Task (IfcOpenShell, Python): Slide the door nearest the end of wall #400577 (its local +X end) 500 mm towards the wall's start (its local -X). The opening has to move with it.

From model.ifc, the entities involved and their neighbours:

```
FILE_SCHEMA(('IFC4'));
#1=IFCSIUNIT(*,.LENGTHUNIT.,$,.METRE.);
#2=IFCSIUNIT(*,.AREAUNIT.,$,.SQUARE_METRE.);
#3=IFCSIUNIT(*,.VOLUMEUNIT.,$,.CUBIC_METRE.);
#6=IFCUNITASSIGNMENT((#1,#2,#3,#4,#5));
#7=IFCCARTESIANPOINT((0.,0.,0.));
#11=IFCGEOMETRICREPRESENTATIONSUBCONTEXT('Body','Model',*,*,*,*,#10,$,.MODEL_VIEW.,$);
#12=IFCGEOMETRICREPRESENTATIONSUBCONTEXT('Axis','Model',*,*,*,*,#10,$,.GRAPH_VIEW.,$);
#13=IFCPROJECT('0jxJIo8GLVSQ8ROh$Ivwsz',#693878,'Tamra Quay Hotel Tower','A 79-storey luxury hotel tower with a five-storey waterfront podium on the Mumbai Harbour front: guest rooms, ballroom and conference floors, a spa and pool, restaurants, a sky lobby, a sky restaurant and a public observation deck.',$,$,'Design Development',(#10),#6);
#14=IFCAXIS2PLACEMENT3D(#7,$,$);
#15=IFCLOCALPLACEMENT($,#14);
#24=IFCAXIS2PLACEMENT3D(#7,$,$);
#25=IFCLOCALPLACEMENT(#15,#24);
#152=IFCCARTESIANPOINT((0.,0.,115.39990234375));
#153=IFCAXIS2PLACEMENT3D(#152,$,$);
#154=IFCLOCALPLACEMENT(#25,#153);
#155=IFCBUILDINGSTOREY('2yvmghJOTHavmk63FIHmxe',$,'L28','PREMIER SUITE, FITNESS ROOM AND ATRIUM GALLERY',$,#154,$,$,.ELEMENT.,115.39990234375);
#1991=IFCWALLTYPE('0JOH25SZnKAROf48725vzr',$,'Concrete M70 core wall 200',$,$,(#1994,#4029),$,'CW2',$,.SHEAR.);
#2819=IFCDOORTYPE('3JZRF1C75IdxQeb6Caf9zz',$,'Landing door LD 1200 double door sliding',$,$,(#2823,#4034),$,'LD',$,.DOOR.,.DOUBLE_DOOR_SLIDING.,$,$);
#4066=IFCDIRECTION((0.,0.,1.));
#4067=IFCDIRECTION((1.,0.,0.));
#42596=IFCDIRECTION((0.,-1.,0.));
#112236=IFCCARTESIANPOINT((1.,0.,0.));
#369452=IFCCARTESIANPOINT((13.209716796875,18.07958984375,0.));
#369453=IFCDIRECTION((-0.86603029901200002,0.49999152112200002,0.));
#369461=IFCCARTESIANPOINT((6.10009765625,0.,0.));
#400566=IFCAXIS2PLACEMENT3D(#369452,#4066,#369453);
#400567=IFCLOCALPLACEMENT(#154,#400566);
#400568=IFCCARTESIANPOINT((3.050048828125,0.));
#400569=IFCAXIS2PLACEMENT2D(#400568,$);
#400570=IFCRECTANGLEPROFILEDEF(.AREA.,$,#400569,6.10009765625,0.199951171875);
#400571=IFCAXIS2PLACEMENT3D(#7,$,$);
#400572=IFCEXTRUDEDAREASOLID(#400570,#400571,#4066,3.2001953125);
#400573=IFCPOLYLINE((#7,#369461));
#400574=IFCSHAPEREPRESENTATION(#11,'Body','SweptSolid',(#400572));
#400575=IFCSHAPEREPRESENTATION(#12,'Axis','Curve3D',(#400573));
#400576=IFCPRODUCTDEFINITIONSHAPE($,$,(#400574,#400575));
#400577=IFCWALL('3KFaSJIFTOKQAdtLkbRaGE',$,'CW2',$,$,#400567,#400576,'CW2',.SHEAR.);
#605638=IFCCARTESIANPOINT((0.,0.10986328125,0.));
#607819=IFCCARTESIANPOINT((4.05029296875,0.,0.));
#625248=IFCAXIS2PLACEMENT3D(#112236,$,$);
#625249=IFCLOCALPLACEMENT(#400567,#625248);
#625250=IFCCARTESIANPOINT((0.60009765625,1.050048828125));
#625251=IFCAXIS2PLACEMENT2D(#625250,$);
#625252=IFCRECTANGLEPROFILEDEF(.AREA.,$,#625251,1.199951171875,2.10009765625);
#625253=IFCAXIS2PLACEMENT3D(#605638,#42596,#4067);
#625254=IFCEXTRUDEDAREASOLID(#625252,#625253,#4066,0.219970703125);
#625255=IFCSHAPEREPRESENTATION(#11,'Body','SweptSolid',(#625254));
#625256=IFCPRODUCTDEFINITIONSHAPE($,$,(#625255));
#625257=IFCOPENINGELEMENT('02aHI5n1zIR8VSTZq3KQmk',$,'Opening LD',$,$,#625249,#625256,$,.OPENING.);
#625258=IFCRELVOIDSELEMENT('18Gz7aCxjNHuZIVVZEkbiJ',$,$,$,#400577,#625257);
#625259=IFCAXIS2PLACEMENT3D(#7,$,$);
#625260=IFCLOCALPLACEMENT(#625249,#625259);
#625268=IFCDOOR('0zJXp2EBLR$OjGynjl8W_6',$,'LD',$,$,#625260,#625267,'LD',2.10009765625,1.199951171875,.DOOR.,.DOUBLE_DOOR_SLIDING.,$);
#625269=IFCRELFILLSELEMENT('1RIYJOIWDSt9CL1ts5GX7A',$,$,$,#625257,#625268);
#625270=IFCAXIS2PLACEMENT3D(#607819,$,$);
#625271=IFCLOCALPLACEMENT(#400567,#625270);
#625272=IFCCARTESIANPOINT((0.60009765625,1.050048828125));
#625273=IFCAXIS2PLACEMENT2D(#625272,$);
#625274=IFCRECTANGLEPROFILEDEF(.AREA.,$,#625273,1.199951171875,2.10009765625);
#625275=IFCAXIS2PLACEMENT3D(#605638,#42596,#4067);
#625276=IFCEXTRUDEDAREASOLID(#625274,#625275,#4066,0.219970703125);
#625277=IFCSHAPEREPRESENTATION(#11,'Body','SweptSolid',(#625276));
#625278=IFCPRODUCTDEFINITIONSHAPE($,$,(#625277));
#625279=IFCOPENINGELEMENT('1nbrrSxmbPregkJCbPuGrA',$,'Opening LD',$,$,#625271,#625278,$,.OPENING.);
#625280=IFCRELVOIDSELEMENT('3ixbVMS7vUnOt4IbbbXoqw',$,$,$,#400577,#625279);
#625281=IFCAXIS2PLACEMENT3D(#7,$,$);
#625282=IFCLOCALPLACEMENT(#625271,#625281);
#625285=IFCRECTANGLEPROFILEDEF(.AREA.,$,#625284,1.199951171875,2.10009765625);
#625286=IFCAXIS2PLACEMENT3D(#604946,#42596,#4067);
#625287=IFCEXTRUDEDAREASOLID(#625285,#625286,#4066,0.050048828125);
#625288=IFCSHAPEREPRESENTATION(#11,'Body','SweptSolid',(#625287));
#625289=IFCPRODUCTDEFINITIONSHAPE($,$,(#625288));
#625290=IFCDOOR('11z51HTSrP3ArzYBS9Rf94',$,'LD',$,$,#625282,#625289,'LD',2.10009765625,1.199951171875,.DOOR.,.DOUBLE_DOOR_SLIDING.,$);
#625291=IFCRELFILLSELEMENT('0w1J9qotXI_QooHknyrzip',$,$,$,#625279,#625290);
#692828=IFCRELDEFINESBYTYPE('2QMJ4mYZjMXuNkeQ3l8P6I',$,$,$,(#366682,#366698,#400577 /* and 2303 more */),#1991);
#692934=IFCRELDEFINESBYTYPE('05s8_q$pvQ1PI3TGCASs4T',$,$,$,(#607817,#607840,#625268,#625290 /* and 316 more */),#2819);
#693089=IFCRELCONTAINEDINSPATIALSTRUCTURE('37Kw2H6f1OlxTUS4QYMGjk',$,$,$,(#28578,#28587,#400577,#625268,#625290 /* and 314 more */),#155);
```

```python
import ifcopenshell
import ifcopenshell.api.geometry
import ifcopenshell.util.placement
import ifcopenshell.util.unit

model = ifcopenshell.open("model.ifc")
unit_scale = ifcopenshell.util.unit.calculate_unit_scale(model)

door = model.by_id(625290)
opening = door.FillsVoids[0].RelatingOpeningElement
wall = opening.VoidsElements[0].RelatingBuildingElement

wall_matrix = ifcopenshell.util.placement.get_local_placement(wall.ObjectPlacement)
shift = wall_matrix[:3, 0] * -0.5 / unit_scale
before = ifcopenshell.util.placement.get_local_placement(door.ObjectPlacement)[:3, 3].copy()

# The door is placed relative to its opening, so it follows when the opening moves.
matrix = ifcopenshell.util.placement.get_local_placement(opening.ObjectPlacement)
matrix[:3, 3] += shift
ifcopenshell.api.geometry.edit_object_placement(
    model, product=opening, matrix=matrix, is_si=False, should_transform_children=True
)

after = ifcopenshell.util.placement.get_local_placement(door.ObjectPlacement)[:3, 3]
print("door moved by", (after - before).round(3) + 0.0)

model.write("model_updated.ifc")
```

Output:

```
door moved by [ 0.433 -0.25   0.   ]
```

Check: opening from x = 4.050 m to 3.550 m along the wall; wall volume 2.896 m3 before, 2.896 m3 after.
